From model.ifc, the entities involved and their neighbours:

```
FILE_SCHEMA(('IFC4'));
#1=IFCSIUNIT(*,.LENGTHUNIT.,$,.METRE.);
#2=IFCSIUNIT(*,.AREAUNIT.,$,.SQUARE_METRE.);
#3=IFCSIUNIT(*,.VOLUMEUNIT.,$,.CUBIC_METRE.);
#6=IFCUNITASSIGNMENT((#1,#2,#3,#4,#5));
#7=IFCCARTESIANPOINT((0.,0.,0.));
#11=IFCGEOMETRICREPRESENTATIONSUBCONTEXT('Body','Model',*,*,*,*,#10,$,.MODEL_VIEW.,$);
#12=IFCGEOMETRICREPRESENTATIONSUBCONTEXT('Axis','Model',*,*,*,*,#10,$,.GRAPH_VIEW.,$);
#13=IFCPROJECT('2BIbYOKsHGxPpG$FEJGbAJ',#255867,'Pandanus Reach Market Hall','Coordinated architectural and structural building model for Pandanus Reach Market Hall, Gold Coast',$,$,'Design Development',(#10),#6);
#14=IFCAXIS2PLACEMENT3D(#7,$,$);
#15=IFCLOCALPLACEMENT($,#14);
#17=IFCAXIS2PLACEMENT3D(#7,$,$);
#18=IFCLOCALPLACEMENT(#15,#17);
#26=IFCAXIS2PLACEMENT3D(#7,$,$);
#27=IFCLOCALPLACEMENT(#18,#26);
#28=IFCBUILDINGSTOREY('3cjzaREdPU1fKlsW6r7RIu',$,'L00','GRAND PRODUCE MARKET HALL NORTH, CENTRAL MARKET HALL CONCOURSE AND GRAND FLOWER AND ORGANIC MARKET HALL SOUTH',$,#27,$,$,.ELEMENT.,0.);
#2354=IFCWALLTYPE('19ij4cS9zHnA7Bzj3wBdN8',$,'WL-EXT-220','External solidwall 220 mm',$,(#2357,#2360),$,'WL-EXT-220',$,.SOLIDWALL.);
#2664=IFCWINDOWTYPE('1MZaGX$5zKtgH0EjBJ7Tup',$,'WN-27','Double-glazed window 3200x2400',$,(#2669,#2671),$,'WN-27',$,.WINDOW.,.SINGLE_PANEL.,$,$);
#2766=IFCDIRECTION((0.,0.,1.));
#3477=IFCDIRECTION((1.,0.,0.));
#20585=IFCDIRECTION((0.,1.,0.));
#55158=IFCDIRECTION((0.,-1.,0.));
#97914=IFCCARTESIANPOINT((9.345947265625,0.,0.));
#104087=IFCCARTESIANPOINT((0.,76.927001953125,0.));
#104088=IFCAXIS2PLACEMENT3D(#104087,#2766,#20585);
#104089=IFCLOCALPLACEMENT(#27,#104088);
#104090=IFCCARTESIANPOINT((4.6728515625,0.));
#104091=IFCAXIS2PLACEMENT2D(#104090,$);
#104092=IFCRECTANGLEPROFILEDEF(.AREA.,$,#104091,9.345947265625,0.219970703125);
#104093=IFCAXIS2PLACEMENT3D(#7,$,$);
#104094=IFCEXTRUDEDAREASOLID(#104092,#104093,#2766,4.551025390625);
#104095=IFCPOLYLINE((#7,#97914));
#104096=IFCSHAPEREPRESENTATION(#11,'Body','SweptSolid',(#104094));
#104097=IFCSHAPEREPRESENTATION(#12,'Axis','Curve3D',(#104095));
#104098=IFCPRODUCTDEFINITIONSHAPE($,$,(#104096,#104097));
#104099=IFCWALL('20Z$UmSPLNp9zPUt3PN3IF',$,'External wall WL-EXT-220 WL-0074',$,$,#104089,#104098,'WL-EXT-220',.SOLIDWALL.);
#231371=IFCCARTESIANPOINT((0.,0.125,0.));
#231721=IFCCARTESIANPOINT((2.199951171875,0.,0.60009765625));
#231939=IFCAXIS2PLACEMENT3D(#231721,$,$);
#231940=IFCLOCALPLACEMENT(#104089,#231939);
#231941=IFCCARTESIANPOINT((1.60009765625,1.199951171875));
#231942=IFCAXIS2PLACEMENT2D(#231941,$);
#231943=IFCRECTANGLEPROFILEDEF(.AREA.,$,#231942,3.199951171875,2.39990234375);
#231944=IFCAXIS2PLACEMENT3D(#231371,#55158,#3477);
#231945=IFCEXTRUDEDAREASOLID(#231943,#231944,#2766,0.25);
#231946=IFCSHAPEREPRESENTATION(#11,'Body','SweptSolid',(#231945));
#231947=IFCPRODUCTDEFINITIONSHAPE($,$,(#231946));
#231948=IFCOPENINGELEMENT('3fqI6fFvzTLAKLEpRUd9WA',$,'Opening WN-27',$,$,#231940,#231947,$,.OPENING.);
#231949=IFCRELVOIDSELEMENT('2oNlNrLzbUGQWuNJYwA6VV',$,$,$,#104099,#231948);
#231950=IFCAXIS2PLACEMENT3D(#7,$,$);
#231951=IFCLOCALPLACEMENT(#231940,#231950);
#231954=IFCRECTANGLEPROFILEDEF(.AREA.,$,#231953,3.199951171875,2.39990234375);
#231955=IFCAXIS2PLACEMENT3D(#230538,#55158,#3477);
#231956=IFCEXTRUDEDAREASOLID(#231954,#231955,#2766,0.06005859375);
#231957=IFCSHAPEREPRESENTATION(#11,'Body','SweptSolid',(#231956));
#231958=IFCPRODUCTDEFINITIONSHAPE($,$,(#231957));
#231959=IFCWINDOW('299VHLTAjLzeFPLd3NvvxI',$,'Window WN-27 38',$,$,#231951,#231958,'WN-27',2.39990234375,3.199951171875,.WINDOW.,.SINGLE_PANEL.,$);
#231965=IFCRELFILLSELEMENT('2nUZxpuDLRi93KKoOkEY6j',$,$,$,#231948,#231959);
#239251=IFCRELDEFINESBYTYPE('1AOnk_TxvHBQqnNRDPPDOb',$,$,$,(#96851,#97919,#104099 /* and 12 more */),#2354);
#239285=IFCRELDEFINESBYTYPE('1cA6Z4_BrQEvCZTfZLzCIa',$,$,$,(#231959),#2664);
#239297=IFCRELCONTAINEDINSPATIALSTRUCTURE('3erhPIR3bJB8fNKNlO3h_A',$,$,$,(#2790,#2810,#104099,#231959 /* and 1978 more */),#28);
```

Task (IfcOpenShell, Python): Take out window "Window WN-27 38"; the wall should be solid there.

```python
import ifcopenshell
import ifcopenshell.api.feature
import ifcopenshell.api.root
import ifcopenshell.geom
import ifcopenshell.util.shape

model = ifcopenshell.open("model.ifc")
settings = ifcopenshell.geom.settings()


def volume(element):
    """Net volume in cubic metres, openings subtracted."""
    shape = ifcopenshell.geom.create_shape(settings, element)
    return ifcopenshell.util.shape.get_volume(shape.geometry)


window = model.by_guid("299VHLTAjLzeFPLd3NvvxI")
opening = window.FillsVoids[0].RelatingOpeningElement
wall = opening.VoidsElements[0].RelatingBuildingElement
before = volume(wall)

ifcopenshell.api.root.remove_product(model, product=window)
ifcopenshell.api.feature.remove_feature(model, feature=opening)

after = volume(wall)

print(f"wall volume {before:.3f} -> {after:.3f} m3")

model.write("model_updated.ifc")
```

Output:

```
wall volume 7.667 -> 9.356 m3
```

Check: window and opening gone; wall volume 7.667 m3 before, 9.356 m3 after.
